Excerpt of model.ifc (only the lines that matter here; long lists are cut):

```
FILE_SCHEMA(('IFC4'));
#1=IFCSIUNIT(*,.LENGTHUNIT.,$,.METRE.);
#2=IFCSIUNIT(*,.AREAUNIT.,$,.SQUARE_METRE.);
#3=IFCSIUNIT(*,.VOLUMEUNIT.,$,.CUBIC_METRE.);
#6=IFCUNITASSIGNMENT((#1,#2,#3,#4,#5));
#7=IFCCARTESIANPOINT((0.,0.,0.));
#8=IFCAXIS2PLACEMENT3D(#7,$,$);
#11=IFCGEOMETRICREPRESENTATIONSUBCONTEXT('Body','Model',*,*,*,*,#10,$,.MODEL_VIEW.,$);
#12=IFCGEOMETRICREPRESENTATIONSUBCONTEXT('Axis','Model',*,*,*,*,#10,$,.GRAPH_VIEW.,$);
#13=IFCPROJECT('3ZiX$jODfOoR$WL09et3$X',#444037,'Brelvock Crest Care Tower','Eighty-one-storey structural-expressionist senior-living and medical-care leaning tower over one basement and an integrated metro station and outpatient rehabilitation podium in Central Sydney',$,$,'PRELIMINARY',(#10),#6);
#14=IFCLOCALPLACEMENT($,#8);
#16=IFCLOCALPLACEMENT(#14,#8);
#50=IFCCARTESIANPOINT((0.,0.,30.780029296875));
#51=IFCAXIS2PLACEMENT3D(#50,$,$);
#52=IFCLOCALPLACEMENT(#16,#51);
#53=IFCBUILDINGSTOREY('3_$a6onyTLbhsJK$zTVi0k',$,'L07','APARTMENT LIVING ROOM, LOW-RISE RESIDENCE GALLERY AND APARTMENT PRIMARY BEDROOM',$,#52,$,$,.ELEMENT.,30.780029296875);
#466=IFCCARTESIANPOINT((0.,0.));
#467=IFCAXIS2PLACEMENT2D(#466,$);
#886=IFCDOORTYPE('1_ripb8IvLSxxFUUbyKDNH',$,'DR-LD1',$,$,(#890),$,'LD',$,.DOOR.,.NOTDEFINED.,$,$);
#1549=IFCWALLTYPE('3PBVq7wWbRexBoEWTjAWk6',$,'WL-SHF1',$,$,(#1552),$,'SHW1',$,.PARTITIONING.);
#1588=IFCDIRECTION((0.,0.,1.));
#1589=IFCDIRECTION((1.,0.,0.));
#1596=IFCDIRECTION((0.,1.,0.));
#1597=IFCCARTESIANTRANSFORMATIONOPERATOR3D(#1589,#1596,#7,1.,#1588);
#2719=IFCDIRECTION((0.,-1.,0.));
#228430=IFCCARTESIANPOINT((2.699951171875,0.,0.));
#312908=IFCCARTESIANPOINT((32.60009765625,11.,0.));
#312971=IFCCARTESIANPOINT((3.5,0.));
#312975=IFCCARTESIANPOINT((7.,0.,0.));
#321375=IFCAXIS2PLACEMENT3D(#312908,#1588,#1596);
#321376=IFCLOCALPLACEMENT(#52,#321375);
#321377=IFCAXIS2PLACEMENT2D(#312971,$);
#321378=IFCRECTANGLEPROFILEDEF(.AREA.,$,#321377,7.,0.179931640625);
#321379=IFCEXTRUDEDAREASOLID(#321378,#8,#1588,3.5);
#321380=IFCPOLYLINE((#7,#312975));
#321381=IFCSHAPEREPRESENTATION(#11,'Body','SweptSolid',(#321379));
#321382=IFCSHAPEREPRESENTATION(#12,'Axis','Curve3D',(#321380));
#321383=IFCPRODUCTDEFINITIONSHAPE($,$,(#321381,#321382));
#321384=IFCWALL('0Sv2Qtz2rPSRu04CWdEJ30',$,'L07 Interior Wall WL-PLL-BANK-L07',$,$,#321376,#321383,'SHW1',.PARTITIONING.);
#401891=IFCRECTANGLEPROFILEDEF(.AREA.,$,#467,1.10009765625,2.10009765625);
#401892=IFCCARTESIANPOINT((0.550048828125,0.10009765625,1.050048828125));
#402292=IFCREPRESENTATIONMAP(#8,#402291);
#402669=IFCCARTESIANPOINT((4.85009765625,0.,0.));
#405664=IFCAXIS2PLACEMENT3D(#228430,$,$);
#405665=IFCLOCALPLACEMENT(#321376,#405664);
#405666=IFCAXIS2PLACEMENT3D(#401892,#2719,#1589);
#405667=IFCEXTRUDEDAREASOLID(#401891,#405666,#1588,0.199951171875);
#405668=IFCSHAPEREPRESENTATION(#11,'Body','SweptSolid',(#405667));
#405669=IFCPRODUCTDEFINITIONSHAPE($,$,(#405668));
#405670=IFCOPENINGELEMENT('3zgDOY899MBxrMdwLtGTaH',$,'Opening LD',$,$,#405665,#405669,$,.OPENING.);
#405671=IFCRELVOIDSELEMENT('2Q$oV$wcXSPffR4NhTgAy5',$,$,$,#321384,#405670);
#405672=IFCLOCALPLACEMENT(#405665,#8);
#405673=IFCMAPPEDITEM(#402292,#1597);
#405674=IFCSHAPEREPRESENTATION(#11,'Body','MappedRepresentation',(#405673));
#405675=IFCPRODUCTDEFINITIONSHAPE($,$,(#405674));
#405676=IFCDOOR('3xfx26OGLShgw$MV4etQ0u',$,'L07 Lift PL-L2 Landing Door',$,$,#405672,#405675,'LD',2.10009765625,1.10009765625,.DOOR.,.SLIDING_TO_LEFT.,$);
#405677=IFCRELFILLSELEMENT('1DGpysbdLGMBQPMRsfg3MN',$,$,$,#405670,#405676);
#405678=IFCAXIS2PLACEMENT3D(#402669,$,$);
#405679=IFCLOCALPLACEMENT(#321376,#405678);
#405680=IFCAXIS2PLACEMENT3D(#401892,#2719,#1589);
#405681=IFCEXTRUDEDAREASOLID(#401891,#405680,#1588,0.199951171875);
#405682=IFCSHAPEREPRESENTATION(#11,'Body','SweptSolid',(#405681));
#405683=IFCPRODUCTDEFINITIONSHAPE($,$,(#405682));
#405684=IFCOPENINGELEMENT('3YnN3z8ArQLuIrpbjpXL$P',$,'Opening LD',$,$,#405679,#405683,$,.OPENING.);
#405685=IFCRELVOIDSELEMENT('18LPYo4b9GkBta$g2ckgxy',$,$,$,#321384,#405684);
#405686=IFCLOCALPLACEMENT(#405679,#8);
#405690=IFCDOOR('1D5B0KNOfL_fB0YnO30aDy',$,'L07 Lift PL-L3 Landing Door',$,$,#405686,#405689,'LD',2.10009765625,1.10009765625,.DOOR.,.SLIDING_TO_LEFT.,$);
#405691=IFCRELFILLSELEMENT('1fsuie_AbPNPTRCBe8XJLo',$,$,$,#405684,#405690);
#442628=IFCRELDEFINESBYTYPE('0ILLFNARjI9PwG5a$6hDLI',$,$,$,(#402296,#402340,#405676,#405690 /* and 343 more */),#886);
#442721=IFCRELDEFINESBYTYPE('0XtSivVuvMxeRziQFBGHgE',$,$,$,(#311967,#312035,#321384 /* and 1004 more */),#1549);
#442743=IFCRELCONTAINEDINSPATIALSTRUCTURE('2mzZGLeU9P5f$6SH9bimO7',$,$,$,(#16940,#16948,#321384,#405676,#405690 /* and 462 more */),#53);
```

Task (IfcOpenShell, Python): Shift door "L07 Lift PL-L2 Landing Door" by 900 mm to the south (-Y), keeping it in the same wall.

```python
import ifcopenshell
import ifcopenshell.api.geometry
import ifcopenshell.util.placement
import ifcopenshell.util.unit

model = ifcopenshell.open("model.ifc")
unit_scale = ifcopenshell.util.unit.calculate_unit_scale(model)

door = model.by_guid("3xfx26OGLShgw$MV4etQ0u")
opening = door.FillsVoids[0].RelatingOpeningElement
wall = opening.VoidsElements[0].RelatingBuildingElement

wall_matrix = ifcopenshell.util.placement.get_local_placement(wall.ObjectPlacement)
shift = wall_matrix[:3, 0] * -0.9 / unit_scale
before = ifcopenshell.util.placement.get_local_placement(door.ObjectPlacement)[:3, 3].copy()

# The door is placed relative to its opening, so it follows when the opening moves.
matrix = ifcopenshell.util.placement.get_local_placement(opening.ObjectPlacement)
matrix[:3, 3] += shift
ifcopenshell.api.geometry.edit_object_placement(
    model, product=opening, matrix=matrix, is_si=False, should_transform_children=True
)

after = ifcopenshell.util.placement.get_local_placement(door.ObjectPlacement)[:3, 3]
print("door moved by", (after - before).round(3) + 0.0)

model.write("model-out.ifc")
```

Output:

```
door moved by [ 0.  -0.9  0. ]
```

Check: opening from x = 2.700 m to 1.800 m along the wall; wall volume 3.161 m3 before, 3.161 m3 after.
